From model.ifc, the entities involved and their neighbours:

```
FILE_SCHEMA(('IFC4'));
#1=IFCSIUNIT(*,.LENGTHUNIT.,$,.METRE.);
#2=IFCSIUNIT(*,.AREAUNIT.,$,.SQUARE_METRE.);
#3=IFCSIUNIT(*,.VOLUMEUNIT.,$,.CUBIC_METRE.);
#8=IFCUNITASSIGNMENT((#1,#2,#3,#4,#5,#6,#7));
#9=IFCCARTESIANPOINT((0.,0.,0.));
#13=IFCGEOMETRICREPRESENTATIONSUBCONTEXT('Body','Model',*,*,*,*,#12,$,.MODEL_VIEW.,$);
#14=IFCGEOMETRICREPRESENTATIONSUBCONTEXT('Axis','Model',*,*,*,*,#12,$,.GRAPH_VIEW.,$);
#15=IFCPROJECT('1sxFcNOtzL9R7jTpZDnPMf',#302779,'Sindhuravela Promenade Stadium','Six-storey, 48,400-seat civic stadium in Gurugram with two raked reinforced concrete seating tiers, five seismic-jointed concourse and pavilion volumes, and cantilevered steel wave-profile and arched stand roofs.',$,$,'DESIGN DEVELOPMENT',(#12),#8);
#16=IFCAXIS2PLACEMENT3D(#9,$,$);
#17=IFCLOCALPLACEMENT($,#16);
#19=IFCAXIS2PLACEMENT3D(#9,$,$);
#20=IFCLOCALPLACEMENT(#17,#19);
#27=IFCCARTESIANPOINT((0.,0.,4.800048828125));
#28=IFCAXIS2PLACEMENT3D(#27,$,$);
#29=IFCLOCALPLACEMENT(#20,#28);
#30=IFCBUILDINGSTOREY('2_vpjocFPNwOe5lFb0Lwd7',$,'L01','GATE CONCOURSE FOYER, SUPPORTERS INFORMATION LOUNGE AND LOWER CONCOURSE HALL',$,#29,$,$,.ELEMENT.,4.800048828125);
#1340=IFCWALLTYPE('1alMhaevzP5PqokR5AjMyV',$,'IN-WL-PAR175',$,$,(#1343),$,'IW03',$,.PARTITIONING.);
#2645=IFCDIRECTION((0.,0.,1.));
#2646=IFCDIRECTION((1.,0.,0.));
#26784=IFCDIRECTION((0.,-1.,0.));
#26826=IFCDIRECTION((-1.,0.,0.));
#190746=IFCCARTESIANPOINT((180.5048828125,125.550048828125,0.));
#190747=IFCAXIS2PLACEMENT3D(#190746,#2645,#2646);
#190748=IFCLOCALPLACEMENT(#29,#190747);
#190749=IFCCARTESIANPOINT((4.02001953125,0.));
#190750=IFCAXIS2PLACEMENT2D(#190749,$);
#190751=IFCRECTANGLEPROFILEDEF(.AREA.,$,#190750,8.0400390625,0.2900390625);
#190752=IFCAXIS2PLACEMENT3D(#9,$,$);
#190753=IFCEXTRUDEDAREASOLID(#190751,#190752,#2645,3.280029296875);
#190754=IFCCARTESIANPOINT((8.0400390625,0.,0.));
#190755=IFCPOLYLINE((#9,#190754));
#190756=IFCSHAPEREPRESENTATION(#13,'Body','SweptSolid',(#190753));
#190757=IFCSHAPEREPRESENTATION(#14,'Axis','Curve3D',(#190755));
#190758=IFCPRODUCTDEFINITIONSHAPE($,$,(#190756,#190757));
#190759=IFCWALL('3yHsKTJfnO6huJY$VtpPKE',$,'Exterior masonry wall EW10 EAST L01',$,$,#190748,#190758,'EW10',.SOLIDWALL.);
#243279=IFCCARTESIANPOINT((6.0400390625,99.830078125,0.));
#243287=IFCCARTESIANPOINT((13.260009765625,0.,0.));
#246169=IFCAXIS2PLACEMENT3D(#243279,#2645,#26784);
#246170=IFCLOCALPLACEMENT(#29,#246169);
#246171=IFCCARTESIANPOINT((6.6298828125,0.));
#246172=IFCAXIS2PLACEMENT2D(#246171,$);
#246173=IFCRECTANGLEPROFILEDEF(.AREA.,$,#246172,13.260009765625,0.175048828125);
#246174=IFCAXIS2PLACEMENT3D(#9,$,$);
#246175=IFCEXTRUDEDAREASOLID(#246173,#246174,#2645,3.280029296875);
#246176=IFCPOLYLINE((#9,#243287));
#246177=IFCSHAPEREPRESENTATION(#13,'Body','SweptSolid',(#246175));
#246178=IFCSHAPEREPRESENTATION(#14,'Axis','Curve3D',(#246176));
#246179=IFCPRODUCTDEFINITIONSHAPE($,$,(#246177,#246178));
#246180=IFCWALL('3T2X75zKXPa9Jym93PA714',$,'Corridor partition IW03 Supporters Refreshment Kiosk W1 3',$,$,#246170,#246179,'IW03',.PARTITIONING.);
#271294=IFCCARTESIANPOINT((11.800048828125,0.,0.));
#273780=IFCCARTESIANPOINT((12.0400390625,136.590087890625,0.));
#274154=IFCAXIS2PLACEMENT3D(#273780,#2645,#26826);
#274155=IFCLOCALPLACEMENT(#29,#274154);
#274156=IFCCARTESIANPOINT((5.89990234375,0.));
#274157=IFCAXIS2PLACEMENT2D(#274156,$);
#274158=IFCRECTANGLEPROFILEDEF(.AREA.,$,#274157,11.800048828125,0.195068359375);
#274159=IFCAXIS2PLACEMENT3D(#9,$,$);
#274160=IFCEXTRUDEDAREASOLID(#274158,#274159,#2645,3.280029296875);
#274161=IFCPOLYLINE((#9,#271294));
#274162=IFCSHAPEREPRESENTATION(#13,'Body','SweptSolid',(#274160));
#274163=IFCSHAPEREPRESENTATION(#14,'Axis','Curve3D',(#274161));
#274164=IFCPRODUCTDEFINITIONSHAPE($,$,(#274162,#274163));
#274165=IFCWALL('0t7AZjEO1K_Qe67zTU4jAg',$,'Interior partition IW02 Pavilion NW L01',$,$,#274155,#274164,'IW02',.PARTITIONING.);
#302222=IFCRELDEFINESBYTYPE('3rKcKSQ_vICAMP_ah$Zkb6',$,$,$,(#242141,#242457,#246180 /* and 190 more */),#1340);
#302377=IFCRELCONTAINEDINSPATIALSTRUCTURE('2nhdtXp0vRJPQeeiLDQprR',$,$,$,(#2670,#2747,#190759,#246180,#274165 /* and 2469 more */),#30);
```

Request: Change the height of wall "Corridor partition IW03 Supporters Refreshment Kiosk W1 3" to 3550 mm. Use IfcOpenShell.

```python
import ifcopenshell
import ifcopenshell.geom
import ifcopenshell.util.representation
import ifcopenshell.util.shape
import ifcopenshell.util.unit

model = ifcopenshell.open("model.ifc")
unit_scale = ifcopenshell.util.unit.calculate_unit_scale(model)
settings = ifcopenshell.geom.settings()


def volume(element):
    """Net volume in cubic metres, openings subtracted."""
    shape = ifcopenshell.geom.create_shape(settings, element)
    return ifcopenshell.util.shape.get_volume(shape.geometry)


wall = model.by_guid("3T2X75zKXPa9Jym93PA714")
before = volume(wall)

body = ifcopenshell.util.representation.get_representation(wall, "Model", "Body")
solid = body.Items[0]
old_height = solid.Depth
solid.Depth = 3.55 / unit_scale
after = volume(wall)

print(f"height {old_height:g} -> {solid.Depth:g}, volume {before:.3f} -> {after:.3f} m3")

model.write("model_rev.ifc")
```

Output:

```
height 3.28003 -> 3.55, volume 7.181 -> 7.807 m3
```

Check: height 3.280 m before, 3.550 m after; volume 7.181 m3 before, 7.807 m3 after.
